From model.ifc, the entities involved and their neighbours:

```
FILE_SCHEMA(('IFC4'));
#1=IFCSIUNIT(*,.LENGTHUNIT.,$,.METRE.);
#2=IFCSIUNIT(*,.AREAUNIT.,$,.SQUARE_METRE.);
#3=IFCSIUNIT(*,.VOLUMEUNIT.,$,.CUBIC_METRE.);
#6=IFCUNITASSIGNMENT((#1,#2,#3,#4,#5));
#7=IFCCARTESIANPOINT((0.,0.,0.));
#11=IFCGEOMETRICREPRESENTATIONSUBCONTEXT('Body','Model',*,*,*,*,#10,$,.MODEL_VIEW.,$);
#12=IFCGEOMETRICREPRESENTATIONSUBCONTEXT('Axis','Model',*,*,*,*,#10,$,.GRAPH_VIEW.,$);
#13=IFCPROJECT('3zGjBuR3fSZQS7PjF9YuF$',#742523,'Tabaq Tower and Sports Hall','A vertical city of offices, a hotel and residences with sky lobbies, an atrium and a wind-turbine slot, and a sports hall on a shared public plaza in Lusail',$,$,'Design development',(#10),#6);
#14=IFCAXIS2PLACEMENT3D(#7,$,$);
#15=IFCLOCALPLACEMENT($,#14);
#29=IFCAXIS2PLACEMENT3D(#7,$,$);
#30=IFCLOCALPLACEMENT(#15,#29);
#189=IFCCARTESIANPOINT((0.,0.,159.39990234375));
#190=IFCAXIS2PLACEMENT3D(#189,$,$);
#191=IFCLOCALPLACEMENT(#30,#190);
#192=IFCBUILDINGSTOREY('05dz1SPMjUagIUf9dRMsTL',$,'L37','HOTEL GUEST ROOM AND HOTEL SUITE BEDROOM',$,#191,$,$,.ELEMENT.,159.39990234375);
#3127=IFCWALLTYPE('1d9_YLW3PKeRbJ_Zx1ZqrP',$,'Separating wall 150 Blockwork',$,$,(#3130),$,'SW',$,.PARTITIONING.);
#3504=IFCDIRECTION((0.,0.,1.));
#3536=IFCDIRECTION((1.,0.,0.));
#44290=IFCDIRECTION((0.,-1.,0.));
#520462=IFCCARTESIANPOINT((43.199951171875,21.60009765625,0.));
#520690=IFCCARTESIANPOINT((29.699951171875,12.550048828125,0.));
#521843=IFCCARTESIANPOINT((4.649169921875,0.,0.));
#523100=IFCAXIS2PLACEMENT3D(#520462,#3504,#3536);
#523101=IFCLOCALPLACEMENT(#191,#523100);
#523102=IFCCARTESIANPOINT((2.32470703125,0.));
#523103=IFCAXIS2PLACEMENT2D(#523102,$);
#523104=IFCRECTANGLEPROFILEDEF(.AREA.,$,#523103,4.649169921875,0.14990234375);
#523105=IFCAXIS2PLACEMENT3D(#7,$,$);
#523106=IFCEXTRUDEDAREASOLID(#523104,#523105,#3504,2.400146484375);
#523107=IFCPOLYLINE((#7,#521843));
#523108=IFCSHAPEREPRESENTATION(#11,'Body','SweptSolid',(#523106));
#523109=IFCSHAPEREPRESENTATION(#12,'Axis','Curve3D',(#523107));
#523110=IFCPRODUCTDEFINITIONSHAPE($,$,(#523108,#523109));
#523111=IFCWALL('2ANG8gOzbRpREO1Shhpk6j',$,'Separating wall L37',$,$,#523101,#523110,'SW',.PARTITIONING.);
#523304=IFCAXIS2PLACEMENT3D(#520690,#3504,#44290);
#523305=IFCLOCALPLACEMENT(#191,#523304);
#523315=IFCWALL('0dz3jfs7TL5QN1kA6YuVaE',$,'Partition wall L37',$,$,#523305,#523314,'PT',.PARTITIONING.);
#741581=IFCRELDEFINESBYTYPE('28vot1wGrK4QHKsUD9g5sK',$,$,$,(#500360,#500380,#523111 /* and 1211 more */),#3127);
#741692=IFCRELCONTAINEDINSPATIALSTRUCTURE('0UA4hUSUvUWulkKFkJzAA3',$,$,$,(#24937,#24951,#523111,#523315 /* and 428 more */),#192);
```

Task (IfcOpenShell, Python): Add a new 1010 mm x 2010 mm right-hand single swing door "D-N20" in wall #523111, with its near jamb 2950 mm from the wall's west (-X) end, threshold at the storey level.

```python
import numpy as np
import ifcopenshell
import ifcopenshell.api.feature
import ifcopenshell.api.geometry
import ifcopenshell.api.root
import ifcopenshell.api.spatial
import ifcopenshell.geom
import ifcopenshell.util.element
import ifcopenshell.util.placement
import ifcopenshell.util.representation
import ifcopenshell.util.shape
import ifcopenshell.util.unit

model = ifcopenshell.open("model.ifc")
unit_scale = ifcopenshell.util.unit.calculate_unit_scale(model)
settings = ifcopenshell.geom.settings()


def volume(element):
    """Net volume in cubic metres, openings subtracted."""
    shape = ifcopenshell.geom.create_shape(settings, element)
    return ifcopenshell.util.shape.get_volume(shape.geometry)


wall = model.by_guid("2ANG8gOzbRpREO1Shhpk6j")
storey = ifcopenshell.util.element.get_container(wall, ifc_class="IfcBuildingStorey")
context = ifcopenshell.util.representation.get_context(model, "Model", "Body", "MODEL_VIEW")
before = volume(wall)

width, height, from_end, sill = 1.01, 2.01, 2.95, 0.0  # metres

# The wall runs along its own X axis, and the end named is its -X end.
wall_shape = ifcopenshell.geom.create_shape(settings, wall)
x, y, z = ifcopenshell.util.shape.get_vertices(wall_shape.geometry).T
start = x.min() + from_end
face, thickness = float(y.min()), float(y.max() - y.min())
wall_matrix = ifcopenshell.util.placement.get_local_placement(wall.ObjectPlacement)
level = ifcopenshell.util.placement.get_local_placement(storey.ObjectPlacement)[2, 3]


def in_wall(x, y):
    """Placement at x, y metres in the wall's axes, at sill height."""
    matrix = wall_matrix.copy()
    matrix[:, 3] = wall_matrix @ np.array([x / unit_scale, y / unit_scale, 0.0, 1.0])
    matrix[2, 3] = level + sill / unit_scale
    return matrix


# Opening: a box that overshoots both wall faces by 50 mm.
opening = ifcopenshell.api.root.create_entity(model, ifc_class="IfcOpeningElement", predefined_type="OPENING")
box = ifcopenshell.api.geometry.add_wall_representation(
    model, context=context, length=width, height=height, thickness=thickness + 0.1
)
ifcopenshell.api.geometry.assign_representation(model, product=opening, representation=box)
ifcopenshell.api.geometry.edit_object_placement(model, product=opening, matrix=in_wall(start, face - 0.05), is_si=False)
ifcopenshell.api.feature.add_feature(model, feature=opening, element=wall)

door = ifcopenshell.api.root.create_entity(model, ifc_class="IfcDoor", name="D-N20", predefined_type="DOOR")
door.OverallWidth, door.OverallHeight = width / unit_scale, height / unit_scale
door.OperationType = "SINGLE_SWING_RIGHT"
body = ifcopenshell.api.geometry.add_door_representation(
    model,
    context=context,
    overall_width=door.OverallWidth,
    overall_height=door.OverallHeight,
    operation_type="SINGLE_SWING_RIGHT",
    lining_properties={"LiningDepth": thickness / unit_scale, "ThresholdDepth": thickness / unit_scale},
)
ifcopenshell.api.geometry.assign_representation(model, product=door, representation=body)
ifcopenshell.api.spatial.assign_container(model, products=[door], relating_structure=storey)
ifcopenshell.api.feature.add_filling(model, opening=opening, element=door)

# The lining spans the wall, so the door starts at the wall face.
ifcopenshell.api.geometry.edit_object_placement(model, product=door, matrix=in_wall(start, face), is_si=False)

after = volume(wall)

print(f"wall volume {before:.3f} -> {after:.3f} m3")

model.write("model_edited.ifc")
```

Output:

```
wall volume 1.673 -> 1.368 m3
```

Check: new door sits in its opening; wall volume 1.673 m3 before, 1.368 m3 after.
